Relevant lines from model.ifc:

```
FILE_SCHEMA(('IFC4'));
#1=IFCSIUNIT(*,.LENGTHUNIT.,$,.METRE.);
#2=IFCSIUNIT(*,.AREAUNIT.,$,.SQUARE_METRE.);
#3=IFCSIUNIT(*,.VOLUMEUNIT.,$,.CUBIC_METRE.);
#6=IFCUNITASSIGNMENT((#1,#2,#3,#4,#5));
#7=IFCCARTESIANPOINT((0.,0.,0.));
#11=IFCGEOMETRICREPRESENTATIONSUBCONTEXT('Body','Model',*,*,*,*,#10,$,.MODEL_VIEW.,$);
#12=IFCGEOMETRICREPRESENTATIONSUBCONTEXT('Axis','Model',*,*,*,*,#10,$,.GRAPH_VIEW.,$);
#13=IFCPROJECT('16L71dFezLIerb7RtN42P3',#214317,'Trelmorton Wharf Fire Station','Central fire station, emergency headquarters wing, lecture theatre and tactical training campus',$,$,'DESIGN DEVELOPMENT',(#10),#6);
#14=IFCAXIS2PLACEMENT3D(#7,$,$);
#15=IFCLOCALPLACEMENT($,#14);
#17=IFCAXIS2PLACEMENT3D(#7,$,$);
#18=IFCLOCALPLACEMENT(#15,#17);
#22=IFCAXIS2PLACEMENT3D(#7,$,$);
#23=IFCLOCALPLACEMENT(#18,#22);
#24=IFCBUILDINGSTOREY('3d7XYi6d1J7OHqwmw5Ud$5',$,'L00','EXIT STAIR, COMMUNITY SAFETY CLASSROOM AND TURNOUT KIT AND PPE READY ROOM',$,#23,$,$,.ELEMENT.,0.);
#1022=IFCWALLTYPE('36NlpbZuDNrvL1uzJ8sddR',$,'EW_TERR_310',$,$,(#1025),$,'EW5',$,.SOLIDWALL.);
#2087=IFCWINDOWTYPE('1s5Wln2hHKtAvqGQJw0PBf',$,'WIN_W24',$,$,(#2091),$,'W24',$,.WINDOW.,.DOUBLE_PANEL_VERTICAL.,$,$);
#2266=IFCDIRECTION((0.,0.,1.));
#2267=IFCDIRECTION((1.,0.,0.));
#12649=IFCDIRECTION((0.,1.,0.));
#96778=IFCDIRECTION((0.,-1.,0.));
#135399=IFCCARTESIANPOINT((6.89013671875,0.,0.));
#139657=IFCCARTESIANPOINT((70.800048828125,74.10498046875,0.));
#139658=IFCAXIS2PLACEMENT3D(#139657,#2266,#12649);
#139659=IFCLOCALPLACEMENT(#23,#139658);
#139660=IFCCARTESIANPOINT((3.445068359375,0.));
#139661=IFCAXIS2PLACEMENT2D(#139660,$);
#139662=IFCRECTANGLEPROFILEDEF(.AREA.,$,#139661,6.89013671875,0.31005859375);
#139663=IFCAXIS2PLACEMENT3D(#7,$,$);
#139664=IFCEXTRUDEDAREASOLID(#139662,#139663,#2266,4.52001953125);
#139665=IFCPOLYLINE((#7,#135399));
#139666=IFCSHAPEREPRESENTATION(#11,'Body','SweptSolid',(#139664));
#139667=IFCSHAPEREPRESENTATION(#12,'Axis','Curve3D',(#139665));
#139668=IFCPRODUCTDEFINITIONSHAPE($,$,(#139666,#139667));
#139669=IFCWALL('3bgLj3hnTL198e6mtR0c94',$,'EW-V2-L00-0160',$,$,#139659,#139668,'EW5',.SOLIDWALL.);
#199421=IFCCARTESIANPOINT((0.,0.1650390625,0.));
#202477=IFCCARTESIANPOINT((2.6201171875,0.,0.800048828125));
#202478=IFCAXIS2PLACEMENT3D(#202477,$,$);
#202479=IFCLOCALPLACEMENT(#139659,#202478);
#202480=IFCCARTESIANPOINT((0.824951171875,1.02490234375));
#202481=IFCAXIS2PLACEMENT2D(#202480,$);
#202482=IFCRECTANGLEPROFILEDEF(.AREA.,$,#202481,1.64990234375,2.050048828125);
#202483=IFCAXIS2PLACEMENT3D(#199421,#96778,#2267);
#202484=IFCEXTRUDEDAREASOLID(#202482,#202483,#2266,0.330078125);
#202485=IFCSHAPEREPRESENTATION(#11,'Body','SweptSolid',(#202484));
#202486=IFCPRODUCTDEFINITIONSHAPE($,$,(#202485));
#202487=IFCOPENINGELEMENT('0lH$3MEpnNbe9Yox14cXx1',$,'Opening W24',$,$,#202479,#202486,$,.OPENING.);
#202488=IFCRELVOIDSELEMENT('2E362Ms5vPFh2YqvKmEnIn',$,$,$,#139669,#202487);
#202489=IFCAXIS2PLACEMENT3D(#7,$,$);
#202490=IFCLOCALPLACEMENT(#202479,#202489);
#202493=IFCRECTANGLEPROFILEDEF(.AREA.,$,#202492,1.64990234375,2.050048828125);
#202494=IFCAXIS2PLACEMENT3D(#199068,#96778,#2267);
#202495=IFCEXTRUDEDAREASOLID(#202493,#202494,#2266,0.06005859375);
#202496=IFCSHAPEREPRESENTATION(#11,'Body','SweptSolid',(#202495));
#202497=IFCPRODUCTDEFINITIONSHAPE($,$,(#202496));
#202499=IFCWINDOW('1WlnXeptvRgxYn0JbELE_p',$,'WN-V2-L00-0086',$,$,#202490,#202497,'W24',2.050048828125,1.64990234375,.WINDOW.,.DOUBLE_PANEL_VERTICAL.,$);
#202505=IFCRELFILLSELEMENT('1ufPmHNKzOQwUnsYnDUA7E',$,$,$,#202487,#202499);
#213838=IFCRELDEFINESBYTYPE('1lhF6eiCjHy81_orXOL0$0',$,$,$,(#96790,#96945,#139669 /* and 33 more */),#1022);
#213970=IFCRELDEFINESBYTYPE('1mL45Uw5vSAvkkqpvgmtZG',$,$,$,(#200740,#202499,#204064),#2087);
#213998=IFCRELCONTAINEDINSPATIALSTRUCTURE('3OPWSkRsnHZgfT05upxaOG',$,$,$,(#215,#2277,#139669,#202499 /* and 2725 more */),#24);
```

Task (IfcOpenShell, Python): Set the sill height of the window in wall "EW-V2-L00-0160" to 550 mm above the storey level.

```python
import numpy as np
import ifcopenshell
import ifcopenshell.api.geometry
import ifcopenshell.geom
import ifcopenshell.util.element
import ifcopenshell.util.placement
import ifcopenshell.util.shape
import ifcopenshell.util.unit

model = ifcopenshell.open("model.ifc")
unit_scale = ifcopenshell.util.unit.calculate_unit_scale(model)

window = model.by_id(202499)
opening = window.FillsVoids[0].RelatingOpeningElement
storey = ifcopenshell.util.element.get_container(window, ifc_class="IfcBuildingStorey")
level = ifcopenshell.util.placement.get_local_placement(storey.ObjectPlacement)[2, 3]

# The opening's origin need not be at the sill, so measure its lowest point.
shape = ifcopenshell.geom.create_shape(ifcopenshell.geom.settings(), opening)
bottom = ifcopenshell.util.shape.get_shape_bottom_elevation(shape, shape.geometry) / unit_scale
dz = level + 0.55 - bottom

shift = np.array([0.0, 0.0, dz])
# The window is placed relative to its opening, so it follows when the opening moves.
matrix = ifcopenshell.util.placement.get_local_placement(opening.ObjectPlacement)
matrix[:3, 3] += shift
ifcopenshell.api.geometry.edit_object_placement(
    model, product=opening, matrix=matrix, is_si=False, should_transform_children=True
)

print(f"moved by {dz * unit_scale:+.3f} m")

model.write("model_updated.ifc")
```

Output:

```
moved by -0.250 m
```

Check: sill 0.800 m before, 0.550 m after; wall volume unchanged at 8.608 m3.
